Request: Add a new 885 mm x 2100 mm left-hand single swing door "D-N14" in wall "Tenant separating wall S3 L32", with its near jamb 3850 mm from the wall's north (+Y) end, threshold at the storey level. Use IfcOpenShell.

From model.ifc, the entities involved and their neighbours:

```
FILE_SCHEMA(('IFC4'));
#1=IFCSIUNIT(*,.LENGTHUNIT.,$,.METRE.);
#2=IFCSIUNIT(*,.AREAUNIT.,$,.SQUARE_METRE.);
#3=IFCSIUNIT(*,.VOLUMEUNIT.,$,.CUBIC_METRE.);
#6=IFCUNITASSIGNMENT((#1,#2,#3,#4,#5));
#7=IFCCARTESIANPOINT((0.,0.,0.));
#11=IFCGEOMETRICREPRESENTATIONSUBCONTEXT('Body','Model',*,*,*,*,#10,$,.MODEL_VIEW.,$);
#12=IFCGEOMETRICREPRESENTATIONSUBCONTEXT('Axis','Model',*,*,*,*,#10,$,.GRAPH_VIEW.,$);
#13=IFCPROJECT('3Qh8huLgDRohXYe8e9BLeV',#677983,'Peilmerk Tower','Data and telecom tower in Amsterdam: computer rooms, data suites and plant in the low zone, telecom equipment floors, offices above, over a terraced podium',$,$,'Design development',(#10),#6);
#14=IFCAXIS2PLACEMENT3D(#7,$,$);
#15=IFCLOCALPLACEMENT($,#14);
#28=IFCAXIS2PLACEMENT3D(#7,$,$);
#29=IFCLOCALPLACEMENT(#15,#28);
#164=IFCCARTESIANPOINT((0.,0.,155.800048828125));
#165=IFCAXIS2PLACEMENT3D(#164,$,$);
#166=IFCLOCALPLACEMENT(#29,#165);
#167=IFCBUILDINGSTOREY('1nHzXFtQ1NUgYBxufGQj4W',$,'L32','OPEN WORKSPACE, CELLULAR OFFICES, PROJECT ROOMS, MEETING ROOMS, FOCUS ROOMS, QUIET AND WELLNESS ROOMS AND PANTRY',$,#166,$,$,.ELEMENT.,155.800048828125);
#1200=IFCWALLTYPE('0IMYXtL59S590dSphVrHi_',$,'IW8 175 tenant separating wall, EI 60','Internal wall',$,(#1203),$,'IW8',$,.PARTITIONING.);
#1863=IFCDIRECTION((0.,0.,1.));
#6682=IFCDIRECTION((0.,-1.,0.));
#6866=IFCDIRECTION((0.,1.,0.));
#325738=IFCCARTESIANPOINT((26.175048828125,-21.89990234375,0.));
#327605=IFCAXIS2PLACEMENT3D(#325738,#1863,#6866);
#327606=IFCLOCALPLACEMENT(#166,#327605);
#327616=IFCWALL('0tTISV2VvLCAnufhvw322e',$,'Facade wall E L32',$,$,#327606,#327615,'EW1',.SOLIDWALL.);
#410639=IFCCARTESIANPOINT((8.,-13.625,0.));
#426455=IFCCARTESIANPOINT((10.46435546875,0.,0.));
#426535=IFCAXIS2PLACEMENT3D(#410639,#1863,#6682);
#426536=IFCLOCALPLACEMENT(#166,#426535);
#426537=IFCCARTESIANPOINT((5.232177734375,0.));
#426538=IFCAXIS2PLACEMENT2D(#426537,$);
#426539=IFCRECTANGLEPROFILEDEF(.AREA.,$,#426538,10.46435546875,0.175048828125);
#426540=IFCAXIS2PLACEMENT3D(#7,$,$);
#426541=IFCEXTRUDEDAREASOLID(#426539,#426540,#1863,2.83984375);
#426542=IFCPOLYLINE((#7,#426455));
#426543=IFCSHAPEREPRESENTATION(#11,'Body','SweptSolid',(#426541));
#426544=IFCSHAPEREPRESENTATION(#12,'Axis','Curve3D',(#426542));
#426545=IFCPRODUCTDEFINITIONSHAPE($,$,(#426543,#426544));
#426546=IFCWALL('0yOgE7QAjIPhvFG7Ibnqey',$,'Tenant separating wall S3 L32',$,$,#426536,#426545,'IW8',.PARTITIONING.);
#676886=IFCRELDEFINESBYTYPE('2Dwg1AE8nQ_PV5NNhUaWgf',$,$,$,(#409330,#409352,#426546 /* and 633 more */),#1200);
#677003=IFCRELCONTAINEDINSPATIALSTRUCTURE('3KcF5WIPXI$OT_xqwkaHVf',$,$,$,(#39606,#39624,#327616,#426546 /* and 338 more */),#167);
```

```python
import numpy as np
import ifcopenshell
import ifcopenshell.api.feature
import ifcopenshell.api.geometry
import ifcopenshell.api.root
import ifcopenshell.api.spatial
import ifcopenshell.geom
import ifcopenshell.util.element
import ifcopenshell.util.placement
import ifcopenshell.util.representation
import ifcopenshell.util.shape
import ifcopenshell.util.unit

model = ifcopenshell.open("model.ifc")
unit_scale = ifcopenshell.util.unit.calculate_unit_scale(model)
settings = ifcopenshell.geom.settings()


def volume(element):
    """Net volume in cubic metres, openings subtracted."""
    shape = ifcopenshell.geom.create_shape(settings, element)
    return ifcopenshell.util.shape.get_volume(shape.geometry)


wall = model.by_id(426546)
storey = ifcopenshell.util.element.get_container(wall, ifc_class="IfcBuildingStorey")
context = ifcopenshell.util.representation.get_context(model, "Model", "Body", "MODEL_VIEW")
before = volume(wall)

width, height, from_end, sill = 0.885, 2.1, 3.85, 0.0  # metres

# The wall runs along its own X axis, and the end named is its -X end.
wall_shape = ifcopenshell.geom.create_shape(settings, wall)
x, y, z = ifcopenshell.util.shape.get_vertices(wall_shape.geometry).T
start = x.min() + from_end
face, thickness = float(y.min()), float(y.max() - y.min())
wall_matrix = ifcopenshell.util.placement.get_local_placement(wall.ObjectPlacement)
level = ifcopenshell.util.placement.get_local_placement(storey.ObjectPlacement)[2, 3]


def in_wall(x, y):
    """Placement at x, y metres in the wall's axes, at sill height."""
    matrix = wall_matrix.copy()
    matrix[:, 3] = wall_matrix @ np.array([x / unit_scale, y / unit_scale, 0.0, 1.0])
    matrix[2, 3] = level + sill / unit_scale
    return matrix


# Opening: a box that overshoots both wall faces by 50 mm.
opening = ifcopenshell.api.root.create_entity(model, ifc_class="IfcOpeningElement", predefined_type="OPENING")
box = ifcopenshell.api.geometry.add_wall_representation(
    model, context=context, length=width, height=height, thickness=thickness + 0.1
)
ifcopenshell.api.geometry.assign_representation(model, product=opening, representation=box)
ifcopenshell.api.geometry.edit_object_placement(model, product=opening, matrix=in_wall(start, face - 0.05), is_si=False)
ifcopenshell.api.feature.add_feature(model, feature=opening, element=wall)

door = ifcopenshell.api.root.create_entity(model, ifc_class="IfcDoor", name="D-N14", predefined_type="DOOR")
door.OverallWidth, door.OverallHeight = width / unit_scale, height / unit_scale
door.OperationType = "SINGLE_SWING_LEFT"
body = ifcopenshell.api.geometry.add_door_representation(
    model,
    context=context,
    overall_width=door.OverallWidth,
    overall_height=door.OverallHeight,
    operation_type="SINGLE_SWING_LEFT",
    lining_properties={"LiningDepth": thickness / unit_scale, "ThresholdDepth": thickness / unit_scale},
)
ifcopenshell.api.geometry.assign_representation(model, product=door, representation=body)
ifcopenshell.api.spatial.assign_container(model, products=[door], relating_structure=storey)
ifcopenshell.api.feature.add_filling(model, opening=opening, element=door)

# The lining spans the wall, so the door starts at the wall face.
ifcopenshell.api.geometry.edit_object_placement(model, product=door, matrix=in_wall(start, face), is_si=False)

after = volume(wall)

print(f"wall volume {before:.3f} -> {after:.3f} m3")

model.write("model_rev.ifc")
```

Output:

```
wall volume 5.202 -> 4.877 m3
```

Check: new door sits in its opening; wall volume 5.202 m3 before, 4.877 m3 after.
